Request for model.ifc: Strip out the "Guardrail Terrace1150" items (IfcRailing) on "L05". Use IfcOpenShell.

First a look at what the model holds.

```python
import ifcopenshell
import ifcopenshell.util.element

model = ifcopenshell.open("model.ifc")
print(model.schema)
storey = next(s for s in model.by_type("IfcBuildingStorey") if s.Name == "L05")
railings = [e for e in ifcopenshell.util.element.get_decomposition(storey) if e.is_a("IfcRailing")]
seen = {}
for e in railings:
    element_type = ifcopenshell.util.element.get_type(e)
    name = element_type.Name if element_type not in (None, e) else None
    seen[name] = seen.get(name, 0) + 1
for name, count in sorted(seen.items(), key=str):
    print(count, "x", name)
```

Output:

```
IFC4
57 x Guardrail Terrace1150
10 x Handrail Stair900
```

```python
import ifcopenshell
import ifcopenshell.api.root
import ifcopenshell.util.element

model = ifcopenshell.open("model.ifc")

storey = next(s for s in model.by_type("IfcBuildingStorey") if s.Name == "L05")
railings = [e for e in ifcopenshell.util.element.get_decomposition(storey) if e.is_a("IfcRailing")]
targets = [e for e in railings if (t := ifcopenshell.util.element.get_type(e)) not in (None, e) and t.Name == "Guardrail Terrace1150"]

for e in targets:
    ifcopenshell.api.root.remove_product(model, product=e)
print(len(targets), "removed")

model.write("model_updated.ifc")
```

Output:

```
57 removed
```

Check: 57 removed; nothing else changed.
